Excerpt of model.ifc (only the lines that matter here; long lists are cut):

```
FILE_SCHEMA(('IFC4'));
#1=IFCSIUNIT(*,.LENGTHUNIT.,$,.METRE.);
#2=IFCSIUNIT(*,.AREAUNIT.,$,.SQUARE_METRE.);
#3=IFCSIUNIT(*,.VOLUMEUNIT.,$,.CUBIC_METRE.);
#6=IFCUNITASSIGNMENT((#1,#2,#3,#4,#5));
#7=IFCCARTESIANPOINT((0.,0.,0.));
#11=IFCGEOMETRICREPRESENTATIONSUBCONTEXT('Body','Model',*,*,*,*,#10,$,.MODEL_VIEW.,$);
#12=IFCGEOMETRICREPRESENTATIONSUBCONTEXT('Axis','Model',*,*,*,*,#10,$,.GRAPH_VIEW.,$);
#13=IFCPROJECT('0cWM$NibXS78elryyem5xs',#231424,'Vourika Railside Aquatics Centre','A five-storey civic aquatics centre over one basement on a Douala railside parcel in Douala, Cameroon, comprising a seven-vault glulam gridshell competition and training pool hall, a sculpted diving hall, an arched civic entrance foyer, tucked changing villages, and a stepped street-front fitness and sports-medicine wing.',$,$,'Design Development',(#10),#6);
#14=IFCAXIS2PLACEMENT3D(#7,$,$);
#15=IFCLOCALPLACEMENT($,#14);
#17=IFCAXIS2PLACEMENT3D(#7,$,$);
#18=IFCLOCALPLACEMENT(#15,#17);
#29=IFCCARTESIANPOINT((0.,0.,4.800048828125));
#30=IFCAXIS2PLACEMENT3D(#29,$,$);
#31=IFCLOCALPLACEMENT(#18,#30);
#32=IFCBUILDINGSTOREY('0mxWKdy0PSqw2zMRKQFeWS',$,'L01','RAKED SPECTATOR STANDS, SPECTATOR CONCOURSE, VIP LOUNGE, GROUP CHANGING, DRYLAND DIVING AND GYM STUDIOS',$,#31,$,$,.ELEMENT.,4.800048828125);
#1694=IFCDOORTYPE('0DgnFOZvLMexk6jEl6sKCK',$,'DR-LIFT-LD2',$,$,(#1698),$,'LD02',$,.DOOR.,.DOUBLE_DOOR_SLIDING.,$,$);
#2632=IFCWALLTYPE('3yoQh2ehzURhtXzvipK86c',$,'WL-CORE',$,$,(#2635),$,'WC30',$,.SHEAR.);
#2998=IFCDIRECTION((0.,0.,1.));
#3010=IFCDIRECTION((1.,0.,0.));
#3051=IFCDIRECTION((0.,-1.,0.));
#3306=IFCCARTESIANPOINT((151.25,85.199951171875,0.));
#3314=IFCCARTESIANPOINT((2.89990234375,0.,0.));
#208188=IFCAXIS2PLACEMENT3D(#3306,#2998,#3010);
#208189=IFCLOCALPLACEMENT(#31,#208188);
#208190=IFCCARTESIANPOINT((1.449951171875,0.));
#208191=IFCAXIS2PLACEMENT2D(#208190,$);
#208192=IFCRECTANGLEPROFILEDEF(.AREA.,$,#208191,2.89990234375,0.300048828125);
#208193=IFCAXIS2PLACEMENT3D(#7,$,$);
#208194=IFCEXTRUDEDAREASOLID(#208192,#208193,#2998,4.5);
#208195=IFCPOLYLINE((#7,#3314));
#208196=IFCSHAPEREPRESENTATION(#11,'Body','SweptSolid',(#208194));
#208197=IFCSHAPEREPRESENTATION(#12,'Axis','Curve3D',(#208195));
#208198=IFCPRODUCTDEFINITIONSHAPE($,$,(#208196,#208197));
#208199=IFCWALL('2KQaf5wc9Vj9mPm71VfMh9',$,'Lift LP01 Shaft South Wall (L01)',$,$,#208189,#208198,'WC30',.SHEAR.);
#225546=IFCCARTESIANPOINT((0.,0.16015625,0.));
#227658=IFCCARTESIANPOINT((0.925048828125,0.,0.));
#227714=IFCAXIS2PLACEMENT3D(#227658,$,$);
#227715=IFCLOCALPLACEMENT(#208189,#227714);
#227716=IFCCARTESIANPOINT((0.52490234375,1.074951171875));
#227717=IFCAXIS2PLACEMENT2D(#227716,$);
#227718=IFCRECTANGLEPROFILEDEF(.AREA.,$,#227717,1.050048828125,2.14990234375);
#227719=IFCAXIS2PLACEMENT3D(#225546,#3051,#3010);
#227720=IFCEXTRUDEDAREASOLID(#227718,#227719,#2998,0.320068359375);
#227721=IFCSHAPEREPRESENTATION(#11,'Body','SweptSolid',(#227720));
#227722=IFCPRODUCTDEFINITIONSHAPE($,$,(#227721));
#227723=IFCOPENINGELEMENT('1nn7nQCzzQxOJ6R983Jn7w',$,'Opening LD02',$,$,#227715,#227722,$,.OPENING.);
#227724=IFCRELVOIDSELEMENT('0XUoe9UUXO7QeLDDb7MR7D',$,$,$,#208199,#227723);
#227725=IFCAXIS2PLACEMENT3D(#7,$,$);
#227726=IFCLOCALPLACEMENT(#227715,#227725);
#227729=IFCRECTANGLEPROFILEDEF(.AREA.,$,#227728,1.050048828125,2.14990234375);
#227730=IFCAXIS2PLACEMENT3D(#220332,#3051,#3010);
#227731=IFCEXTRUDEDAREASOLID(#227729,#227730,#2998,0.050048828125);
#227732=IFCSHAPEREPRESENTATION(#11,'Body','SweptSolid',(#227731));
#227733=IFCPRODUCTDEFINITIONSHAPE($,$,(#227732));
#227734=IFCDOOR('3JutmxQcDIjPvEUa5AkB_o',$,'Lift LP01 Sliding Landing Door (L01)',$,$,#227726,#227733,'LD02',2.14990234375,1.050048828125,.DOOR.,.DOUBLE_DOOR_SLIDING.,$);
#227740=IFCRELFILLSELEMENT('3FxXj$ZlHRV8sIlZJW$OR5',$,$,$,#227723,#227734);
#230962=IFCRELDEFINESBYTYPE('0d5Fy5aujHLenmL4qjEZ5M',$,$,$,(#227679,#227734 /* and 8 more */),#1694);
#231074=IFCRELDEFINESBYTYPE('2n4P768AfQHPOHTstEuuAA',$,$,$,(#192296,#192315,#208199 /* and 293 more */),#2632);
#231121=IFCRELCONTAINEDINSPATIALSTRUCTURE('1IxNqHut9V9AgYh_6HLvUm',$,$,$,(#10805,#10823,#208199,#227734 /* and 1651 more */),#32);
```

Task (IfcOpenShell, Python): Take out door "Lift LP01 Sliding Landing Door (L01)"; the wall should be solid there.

```python
import ifcopenshell
import ifcopenshell.api.feature
import ifcopenshell.api.root
import ifcopenshell.geom
import ifcopenshell.util.shape

model = ifcopenshell.open("model.ifc")
settings = ifcopenshell.geom.settings()


def volume(element):
    """Net volume in cubic metres, openings subtracted."""
    shape = ifcopenshell.geom.create_shape(settings, element)
    return ifcopenshell.util.shape.get_volume(shape.geometry)


door = model.by_guid("3JutmxQcDIjPvEUa5AkB_o")
opening = door.FillsVoids[0].RelatingOpeningElement
wall = opening.VoidsElements[0].RelatingBuildingElement
before = volume(wall)

ifcopenshell.api.root.remove_product(model, product=door)
ifcopenshell.api.feature.remove_feature(model, feature=opening)

after = volume(wall)

print(f"wall volume {before:.3f} -> {after:.3f} m3")

model.write("model_v2.ifc")
```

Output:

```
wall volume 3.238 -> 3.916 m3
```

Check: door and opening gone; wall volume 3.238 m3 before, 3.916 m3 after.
